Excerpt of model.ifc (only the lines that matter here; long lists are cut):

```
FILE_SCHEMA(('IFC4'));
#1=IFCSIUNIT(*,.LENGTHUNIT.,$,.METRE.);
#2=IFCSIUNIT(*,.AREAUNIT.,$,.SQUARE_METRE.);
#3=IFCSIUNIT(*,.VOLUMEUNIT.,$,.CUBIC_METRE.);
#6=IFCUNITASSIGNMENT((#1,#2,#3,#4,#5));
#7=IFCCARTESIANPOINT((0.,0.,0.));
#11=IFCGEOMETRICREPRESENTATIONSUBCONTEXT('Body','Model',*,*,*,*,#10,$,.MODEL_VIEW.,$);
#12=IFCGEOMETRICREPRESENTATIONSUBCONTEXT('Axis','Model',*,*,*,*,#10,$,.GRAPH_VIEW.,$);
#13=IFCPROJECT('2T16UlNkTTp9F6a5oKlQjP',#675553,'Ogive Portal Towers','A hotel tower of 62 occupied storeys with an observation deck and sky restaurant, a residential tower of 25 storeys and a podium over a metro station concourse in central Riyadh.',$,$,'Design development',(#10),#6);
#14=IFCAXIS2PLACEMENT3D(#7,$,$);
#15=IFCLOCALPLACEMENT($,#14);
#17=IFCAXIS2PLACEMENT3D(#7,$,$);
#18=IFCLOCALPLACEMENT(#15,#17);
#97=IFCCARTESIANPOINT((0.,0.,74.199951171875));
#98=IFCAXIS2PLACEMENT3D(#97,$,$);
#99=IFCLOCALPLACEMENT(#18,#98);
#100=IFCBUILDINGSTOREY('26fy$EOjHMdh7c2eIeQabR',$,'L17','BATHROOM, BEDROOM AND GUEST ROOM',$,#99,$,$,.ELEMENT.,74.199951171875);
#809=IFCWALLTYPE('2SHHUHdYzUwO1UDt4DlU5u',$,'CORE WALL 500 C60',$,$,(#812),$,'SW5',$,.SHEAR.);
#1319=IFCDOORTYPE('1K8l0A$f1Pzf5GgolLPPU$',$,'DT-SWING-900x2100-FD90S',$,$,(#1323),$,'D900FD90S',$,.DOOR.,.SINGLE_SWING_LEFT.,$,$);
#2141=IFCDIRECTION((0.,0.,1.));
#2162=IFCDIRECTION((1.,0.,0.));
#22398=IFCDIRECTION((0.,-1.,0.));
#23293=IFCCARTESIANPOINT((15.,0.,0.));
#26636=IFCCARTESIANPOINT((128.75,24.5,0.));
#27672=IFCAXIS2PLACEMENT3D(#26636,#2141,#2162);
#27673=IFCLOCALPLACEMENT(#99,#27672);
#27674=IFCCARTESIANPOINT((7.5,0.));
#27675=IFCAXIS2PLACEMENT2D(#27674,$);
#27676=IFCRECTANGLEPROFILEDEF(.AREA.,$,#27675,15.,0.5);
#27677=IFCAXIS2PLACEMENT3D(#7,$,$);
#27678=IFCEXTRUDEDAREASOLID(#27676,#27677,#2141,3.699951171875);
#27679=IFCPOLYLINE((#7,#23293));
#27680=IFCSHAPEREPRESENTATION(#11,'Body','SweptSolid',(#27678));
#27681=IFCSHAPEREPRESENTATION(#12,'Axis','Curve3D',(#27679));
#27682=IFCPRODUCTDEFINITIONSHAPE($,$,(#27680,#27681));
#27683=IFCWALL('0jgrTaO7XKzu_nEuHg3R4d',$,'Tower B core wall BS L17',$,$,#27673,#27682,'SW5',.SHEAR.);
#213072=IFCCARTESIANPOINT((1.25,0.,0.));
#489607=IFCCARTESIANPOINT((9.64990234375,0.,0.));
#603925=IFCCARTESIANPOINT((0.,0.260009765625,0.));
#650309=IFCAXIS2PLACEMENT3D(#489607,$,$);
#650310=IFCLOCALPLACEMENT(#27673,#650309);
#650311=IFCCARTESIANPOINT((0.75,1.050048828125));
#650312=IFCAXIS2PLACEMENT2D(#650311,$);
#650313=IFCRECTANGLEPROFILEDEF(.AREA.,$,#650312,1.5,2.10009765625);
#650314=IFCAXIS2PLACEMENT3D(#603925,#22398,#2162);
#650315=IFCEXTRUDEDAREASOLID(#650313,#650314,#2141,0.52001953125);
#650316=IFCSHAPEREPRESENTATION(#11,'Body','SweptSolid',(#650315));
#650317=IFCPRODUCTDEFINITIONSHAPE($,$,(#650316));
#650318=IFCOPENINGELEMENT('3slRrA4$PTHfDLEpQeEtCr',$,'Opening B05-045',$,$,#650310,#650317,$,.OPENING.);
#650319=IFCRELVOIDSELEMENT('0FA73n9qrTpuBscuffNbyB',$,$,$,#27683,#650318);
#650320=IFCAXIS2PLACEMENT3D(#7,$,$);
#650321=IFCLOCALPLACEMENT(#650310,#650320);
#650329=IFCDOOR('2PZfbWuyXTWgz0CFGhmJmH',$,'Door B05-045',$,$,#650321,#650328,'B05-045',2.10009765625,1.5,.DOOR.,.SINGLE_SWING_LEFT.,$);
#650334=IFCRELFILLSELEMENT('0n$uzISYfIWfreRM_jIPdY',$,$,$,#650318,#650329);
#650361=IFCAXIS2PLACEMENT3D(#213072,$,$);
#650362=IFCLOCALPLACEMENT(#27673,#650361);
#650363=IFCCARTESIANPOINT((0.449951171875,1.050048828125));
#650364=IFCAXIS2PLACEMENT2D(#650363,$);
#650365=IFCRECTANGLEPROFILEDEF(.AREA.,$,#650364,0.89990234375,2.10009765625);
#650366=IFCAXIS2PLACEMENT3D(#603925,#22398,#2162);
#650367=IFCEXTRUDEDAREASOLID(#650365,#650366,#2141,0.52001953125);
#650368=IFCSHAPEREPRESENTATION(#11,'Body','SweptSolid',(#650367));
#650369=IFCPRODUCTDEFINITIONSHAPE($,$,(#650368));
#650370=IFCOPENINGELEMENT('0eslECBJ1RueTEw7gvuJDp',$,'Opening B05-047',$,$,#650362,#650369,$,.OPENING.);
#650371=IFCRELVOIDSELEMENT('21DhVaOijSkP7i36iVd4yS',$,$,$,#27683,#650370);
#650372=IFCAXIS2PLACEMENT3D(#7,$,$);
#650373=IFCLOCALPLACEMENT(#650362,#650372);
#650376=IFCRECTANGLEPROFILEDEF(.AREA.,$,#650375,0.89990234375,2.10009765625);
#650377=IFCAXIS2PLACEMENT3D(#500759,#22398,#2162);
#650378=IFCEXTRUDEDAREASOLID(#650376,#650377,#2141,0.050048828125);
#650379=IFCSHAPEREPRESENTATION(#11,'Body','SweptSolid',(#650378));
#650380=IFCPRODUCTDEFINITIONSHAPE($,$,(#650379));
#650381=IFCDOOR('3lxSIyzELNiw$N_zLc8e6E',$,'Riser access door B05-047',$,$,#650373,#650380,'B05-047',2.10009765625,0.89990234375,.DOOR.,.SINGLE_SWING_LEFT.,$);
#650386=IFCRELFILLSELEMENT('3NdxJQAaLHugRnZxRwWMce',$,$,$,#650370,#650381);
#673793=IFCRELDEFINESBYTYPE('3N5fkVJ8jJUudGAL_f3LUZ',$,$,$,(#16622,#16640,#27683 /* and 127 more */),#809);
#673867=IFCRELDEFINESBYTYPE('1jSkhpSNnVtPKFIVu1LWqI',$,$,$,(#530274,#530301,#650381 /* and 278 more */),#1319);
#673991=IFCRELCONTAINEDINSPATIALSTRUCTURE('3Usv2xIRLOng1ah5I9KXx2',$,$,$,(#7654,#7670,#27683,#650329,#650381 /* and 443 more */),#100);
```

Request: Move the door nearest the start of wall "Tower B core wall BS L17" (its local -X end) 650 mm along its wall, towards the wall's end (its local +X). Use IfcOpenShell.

```python
import ifcopenshell
import ifcopenshell.api.geometry
import ifcopenshell.util.placement
import ifcopenshell.util.unit

model = ifcopenshell.open("model.ifc")
unit_scale = ifcopenshell.util.unit.calculate_unit_scale(model)

door = model.by_id(650381)
opening = door.FillsVoids[0].RelatingOpeningElement
wall = opening.VoidsElements[0].RelatingBuildingElement

wall_matrix = ifcopenshell.util.placement.get_local_placement(wall.ObjectPlacement)
shift = wall_matrix[:3, 0] * 0.65 / unit_scale
before = ifcopenshell.util.placement.get_local_placement(door.ObjectPlacement)[:3, 3].copy()

# The door is placed relative to its opening, so it follows when the opening moves.
matrix = ifcopenshell.util.placement.get_local_placement(opening.ObjectPlacement)
matrix[:3, 3] += shift
ifcopenshell.api.geometry.edit_object_placement(
    model, product=opening, matrix=matrix, is_si=False, should_transform_children=True
)

after = ifcopenshell.util.placement.get_local_placement(door.ObjectPlacement)[:3, 3]
print("door moved by", (after - before).round(3) + 0.0)

model.write("model_updated.ifc")
```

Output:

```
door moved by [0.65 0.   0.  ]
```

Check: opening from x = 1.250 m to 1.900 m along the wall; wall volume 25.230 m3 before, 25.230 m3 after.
